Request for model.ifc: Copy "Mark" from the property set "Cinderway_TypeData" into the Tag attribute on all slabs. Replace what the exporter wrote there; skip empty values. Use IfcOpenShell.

First a look at what the model holds.

```python
import ifcopenshell
import ifcopenshell.util.element

model = ifcopenshell.open("model.ifc")
print(model.schema)
slabs = model.by_type("IfcSlab")
print(len(slabs), "slabs")
for e in slabs[:8]:
    source = ifcopenshell.util.element.get_pset(e, "Cinderway_TypeData", "Mark")
    target = e.Tag
    print(e.id(), repr(source), repr(target), sep=" | ")
```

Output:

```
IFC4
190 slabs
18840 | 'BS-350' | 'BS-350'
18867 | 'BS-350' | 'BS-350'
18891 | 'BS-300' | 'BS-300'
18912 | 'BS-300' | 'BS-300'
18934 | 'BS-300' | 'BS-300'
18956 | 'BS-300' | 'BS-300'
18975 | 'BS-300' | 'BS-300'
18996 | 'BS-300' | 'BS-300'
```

```python
import ifcopenshell
import ifcopenshell.util.element

model = ifcopenshell.open("model.ifc")

count = 0
for e in model.by_type("IfcSlab"):
    value = ifcopenshell.util.element.get_pset(e, "Cinderway_TypeData", "Mark")
    current = e.Tag
    if not value or not value.strip() or current == value:
        continue
    e.Tag = value
    count += 1

print(count, "slabs updated")

model.write("model-out.ifc")
```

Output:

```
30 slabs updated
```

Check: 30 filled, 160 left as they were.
